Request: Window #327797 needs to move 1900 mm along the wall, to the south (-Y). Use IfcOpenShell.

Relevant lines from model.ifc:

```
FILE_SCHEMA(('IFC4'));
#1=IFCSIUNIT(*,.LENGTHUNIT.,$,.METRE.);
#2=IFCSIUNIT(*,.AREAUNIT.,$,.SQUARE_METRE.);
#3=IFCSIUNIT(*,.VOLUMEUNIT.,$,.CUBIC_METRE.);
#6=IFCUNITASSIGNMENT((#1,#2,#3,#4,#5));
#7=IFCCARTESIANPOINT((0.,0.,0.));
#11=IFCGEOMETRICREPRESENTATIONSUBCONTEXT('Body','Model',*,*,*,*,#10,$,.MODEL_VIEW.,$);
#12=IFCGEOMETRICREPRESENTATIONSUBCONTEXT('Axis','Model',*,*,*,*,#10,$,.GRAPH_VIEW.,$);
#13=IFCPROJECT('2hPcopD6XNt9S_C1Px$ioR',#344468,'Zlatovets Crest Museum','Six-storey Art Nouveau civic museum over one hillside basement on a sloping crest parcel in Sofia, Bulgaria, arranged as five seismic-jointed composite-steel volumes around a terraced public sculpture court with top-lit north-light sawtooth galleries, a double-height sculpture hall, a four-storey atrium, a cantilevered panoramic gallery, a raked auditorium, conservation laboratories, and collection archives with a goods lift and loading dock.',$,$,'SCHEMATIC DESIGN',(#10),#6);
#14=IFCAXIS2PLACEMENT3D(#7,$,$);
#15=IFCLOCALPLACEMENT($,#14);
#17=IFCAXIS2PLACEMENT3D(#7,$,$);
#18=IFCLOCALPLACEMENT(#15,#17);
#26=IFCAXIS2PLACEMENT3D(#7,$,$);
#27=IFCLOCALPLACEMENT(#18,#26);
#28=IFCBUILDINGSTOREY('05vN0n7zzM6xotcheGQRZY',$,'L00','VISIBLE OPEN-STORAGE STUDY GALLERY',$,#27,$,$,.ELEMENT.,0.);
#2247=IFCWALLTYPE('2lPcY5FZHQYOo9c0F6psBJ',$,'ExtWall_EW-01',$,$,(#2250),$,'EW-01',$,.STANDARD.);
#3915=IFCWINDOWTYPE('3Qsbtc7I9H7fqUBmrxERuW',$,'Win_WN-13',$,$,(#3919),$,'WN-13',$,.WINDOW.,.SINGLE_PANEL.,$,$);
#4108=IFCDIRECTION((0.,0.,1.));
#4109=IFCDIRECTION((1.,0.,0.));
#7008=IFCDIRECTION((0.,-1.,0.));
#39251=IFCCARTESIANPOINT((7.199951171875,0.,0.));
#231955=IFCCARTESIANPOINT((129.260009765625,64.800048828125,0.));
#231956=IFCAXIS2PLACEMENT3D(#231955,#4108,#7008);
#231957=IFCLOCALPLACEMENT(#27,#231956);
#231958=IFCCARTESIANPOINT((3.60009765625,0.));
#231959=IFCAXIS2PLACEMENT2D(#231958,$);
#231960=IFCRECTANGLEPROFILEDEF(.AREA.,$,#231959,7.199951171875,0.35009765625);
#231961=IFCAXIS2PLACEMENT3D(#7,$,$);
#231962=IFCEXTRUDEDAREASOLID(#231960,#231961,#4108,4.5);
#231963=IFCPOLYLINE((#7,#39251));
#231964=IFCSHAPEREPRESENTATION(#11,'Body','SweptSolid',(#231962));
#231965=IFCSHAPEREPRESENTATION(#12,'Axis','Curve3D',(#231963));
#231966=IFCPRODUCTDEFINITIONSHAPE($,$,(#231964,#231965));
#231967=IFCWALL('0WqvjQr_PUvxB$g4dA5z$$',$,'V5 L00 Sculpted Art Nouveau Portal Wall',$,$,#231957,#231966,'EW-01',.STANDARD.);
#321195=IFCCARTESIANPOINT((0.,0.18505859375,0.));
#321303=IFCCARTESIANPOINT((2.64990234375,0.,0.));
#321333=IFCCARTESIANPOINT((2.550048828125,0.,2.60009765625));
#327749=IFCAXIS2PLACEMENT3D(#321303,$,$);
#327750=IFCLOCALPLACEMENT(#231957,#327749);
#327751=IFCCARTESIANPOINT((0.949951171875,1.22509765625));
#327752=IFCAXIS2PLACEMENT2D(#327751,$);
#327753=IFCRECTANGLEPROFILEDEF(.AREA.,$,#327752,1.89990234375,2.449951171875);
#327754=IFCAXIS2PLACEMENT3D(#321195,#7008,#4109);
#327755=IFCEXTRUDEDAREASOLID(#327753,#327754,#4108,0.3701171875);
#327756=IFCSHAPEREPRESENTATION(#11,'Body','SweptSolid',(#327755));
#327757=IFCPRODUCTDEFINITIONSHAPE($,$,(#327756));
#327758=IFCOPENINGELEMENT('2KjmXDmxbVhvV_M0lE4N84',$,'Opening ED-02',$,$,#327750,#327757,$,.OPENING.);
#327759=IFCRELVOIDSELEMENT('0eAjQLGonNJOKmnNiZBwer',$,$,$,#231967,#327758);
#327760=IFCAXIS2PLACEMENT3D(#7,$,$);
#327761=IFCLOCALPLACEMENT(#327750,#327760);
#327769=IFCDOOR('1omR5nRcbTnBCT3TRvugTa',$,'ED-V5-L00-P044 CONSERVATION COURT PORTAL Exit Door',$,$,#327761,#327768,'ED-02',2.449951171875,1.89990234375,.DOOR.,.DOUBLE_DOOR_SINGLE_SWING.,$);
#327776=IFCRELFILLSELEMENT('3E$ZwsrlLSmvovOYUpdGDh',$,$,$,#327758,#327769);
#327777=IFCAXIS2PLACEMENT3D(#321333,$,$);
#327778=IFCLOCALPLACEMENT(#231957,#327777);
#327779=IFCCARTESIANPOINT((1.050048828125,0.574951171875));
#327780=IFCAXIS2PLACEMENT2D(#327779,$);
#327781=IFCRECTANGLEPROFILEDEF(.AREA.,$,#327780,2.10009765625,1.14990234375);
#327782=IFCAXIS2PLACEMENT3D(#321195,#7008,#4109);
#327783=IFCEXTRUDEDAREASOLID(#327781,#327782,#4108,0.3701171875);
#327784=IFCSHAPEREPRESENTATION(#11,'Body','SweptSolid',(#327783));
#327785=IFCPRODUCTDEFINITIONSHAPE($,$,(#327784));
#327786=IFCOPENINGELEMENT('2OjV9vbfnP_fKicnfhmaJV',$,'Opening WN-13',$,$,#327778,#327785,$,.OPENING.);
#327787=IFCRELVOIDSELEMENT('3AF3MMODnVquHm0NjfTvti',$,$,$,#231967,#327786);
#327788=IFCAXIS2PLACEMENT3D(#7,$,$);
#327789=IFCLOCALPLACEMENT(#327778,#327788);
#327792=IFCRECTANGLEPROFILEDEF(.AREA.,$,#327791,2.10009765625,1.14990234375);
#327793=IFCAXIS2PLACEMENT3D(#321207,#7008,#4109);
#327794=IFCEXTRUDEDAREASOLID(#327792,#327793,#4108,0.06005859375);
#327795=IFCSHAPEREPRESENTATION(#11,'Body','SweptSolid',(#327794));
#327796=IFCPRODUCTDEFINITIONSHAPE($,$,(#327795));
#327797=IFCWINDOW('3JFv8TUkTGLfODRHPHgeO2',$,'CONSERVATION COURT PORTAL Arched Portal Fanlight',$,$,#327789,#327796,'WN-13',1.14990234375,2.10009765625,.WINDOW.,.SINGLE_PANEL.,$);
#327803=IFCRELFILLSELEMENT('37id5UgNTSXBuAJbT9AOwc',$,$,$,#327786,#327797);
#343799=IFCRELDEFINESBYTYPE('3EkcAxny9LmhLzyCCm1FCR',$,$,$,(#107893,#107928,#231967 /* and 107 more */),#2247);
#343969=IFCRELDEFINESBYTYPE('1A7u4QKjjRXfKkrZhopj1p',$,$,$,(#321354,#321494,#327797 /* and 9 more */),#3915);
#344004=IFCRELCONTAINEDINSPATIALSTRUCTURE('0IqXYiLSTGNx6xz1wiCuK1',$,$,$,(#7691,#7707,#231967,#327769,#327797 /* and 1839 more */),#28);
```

```python
import ifcopenshell
import ifcopenshell.api.geometry
import ifcopenshell.util.placement
import ifcopenshell.util.unit

model = ifcopenshell.open("model.ifc")
unit_scale = ifcopenshell.util.unit.calculate_unit_scale(model)

window = model.by_guid("3JFv8TUkTGLfODRHPHgeO2")
opening = window.FillsVoids[0].RelatingOpeningElement
wall = opening.VoidsElements[0].RelatingBuildingElement

wall_matrix = ifcopenshell.util.placement.get_local_placement(wall.ObjectPlacement)
shift = wall_matrix[:3, 0] * 1.9 / unit_scale
before = ifcopenshell.util.placement.get_local_placement(window.ObjectPlacement)[:3, 3].copy()

# The window is placed relative to its opening, so it follows when the opening moves.
matrix = ifcopenshell.util.placement.get_local_placement(opening.ObjectPlacement)
matrix[:3, 3] += shift
ifcopenshell.api.geometry.edit_object_placement(
    model, product=opening, matrix=matrix, is_si=False, should_transform_children=True
)

after = ifcopenshell.util.placement.get_local_placement(window.ObjectPlacement)[:3, 3]
print("window moved by", (after - before).round(3) + 0.0)

model.write("model_rev.ifc")
```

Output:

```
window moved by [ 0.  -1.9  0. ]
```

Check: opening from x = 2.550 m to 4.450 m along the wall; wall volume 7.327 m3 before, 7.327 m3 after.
